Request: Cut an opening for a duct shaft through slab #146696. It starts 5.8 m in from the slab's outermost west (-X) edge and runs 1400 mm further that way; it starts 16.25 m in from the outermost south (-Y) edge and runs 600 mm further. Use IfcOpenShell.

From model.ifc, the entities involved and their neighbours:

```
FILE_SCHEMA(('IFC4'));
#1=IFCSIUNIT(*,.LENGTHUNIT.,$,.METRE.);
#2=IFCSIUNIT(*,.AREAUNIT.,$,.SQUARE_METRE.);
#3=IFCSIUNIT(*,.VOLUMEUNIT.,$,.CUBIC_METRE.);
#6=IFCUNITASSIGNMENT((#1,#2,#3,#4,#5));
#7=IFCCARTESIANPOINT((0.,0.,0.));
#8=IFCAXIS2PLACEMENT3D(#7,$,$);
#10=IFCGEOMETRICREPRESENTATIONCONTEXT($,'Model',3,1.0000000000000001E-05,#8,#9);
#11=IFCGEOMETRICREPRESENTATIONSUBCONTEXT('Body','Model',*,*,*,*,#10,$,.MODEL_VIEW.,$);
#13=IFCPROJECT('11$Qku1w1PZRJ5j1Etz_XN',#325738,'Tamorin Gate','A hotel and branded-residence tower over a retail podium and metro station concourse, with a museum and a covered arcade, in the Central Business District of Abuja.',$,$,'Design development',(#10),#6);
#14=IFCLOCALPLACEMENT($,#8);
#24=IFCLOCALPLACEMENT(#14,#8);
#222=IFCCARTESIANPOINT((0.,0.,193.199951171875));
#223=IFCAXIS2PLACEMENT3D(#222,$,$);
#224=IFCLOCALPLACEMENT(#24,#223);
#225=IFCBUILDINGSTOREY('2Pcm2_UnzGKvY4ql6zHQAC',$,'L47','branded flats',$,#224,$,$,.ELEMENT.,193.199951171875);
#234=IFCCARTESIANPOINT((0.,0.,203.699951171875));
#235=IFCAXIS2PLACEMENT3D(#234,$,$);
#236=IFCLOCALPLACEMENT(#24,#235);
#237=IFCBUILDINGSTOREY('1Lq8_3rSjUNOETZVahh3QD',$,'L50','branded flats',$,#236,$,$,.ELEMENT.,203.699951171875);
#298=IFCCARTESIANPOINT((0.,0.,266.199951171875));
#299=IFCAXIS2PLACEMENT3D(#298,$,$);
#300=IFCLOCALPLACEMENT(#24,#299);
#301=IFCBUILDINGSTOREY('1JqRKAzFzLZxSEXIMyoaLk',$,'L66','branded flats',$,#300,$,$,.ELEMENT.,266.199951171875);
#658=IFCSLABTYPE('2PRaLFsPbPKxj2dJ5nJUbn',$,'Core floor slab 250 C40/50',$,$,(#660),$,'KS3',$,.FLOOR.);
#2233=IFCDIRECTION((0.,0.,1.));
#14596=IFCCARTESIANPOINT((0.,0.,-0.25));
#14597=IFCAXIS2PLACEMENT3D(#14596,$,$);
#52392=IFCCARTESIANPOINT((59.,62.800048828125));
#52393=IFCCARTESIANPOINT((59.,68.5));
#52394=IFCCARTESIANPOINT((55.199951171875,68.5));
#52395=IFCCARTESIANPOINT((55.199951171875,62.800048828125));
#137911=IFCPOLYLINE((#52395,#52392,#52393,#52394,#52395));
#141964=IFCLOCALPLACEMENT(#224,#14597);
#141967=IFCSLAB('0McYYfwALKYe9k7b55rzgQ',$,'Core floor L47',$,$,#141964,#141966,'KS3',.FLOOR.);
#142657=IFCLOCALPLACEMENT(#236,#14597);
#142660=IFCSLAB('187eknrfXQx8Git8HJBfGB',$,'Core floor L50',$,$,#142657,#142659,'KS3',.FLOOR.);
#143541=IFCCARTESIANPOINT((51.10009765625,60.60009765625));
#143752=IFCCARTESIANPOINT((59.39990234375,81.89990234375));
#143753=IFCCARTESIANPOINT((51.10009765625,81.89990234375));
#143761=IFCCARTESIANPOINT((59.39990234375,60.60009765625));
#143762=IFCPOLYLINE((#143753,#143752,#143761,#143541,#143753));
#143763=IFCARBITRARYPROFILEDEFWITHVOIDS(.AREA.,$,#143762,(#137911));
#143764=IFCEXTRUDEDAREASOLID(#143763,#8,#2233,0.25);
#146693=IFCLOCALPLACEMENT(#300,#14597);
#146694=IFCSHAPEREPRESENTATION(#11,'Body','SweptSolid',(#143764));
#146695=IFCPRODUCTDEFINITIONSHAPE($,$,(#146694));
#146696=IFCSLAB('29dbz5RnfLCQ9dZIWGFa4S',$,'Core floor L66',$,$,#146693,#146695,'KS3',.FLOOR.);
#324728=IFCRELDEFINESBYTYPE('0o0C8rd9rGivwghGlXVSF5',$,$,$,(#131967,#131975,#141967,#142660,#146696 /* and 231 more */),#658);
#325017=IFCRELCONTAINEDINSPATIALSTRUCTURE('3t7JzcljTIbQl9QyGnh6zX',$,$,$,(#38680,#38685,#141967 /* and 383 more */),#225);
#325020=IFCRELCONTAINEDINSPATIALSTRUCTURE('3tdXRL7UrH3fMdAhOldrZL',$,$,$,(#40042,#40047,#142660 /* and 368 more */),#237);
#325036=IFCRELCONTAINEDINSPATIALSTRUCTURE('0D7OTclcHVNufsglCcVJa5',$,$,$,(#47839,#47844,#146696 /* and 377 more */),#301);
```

```python
import numpy as np
import ifcopenshell
import ifcopenshell.api.feature
import ifcopenshell.api.geometry
import ifcopenshell.api.root
import ifcopenshell.geom
import ifcopenshell.util.placement
import ifcopenshell.util.representation
import ifcopenshell.util.shape
import ifcopenshell.util.unit

model = ifcopenshell.open("model.ifc")
unit_scale = ifcopenshell.util.unit.calculate_unit_scale(model)
settings = ifcopenshell.geom.settings()


def volume(element):
    """Net volume in cubic metres, openings subtracted."""
    shape = ifcopenshell.geom.create_shape(settings, element)
    return ifcopenshell.util.shape.get_volume(shape.geometry)


slab = model.by_guid("29dbz5RnfLCQ9dZIWGFa4S")
before = volume(slab)

# Extent in the slab's own axes, in metres. The edges named are its -X and -Y sides.
slab_shape = ifcopenshell.geom.create_shape(settings, slab)
vertices = ifcopenshell.util.shape.get_vertices(slab_shape.geometry)
x_min, y_min, bottom = vertices.min(axis=0)
top = vertices[:, 2].max()

opening = ifcopenshell.api.root.create_entity(model, ifc_class="IfcOpeningElement", name="Duct shaft opening", predefined_type="OPENING")
context = ifcopenshell.util.representation.get_context(model, "Model", "Body", "MODEL_VIEW")
width, depth = 1.4, 0.6
outline = [(0.0, 0.0), (width, 0.0), (width, depth), (0.0, depth), (0.0, 0.0)]
# Overshoot both faces by 50 mm so the cut is clean.
shape = ifcopenshell.api.geometry.add_slab_representation(
    model, context=context, depth=top - bottom + 0.1, polyline=outline
)
ifcopenshell.api.geometry.assign_representation(model, product=opening, representation=shape)

matrix = ifcopenshell.util.placement.get_local_placement(slab.ObjectPlacement)
matrix[:, 3] = matrix @ np.append(np.array([x_min + 5.8, y_min + 16.25, bottom - 0.05]) / unit_scale, 1.0)
ifcopenshell.api.geometry.edit_object_placement(model, product=opening, matrix=matrix, is_si=False)
ifcopenshell.api.feature.add_feature(model, feature=opening, element=slab)

after = volume(slab)

print(f"slab volume {before:.3f} -> {after:.3f} m3")

model.write("model_edited.ifc")
```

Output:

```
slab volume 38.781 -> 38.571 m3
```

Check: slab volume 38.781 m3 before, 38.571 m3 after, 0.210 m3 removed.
